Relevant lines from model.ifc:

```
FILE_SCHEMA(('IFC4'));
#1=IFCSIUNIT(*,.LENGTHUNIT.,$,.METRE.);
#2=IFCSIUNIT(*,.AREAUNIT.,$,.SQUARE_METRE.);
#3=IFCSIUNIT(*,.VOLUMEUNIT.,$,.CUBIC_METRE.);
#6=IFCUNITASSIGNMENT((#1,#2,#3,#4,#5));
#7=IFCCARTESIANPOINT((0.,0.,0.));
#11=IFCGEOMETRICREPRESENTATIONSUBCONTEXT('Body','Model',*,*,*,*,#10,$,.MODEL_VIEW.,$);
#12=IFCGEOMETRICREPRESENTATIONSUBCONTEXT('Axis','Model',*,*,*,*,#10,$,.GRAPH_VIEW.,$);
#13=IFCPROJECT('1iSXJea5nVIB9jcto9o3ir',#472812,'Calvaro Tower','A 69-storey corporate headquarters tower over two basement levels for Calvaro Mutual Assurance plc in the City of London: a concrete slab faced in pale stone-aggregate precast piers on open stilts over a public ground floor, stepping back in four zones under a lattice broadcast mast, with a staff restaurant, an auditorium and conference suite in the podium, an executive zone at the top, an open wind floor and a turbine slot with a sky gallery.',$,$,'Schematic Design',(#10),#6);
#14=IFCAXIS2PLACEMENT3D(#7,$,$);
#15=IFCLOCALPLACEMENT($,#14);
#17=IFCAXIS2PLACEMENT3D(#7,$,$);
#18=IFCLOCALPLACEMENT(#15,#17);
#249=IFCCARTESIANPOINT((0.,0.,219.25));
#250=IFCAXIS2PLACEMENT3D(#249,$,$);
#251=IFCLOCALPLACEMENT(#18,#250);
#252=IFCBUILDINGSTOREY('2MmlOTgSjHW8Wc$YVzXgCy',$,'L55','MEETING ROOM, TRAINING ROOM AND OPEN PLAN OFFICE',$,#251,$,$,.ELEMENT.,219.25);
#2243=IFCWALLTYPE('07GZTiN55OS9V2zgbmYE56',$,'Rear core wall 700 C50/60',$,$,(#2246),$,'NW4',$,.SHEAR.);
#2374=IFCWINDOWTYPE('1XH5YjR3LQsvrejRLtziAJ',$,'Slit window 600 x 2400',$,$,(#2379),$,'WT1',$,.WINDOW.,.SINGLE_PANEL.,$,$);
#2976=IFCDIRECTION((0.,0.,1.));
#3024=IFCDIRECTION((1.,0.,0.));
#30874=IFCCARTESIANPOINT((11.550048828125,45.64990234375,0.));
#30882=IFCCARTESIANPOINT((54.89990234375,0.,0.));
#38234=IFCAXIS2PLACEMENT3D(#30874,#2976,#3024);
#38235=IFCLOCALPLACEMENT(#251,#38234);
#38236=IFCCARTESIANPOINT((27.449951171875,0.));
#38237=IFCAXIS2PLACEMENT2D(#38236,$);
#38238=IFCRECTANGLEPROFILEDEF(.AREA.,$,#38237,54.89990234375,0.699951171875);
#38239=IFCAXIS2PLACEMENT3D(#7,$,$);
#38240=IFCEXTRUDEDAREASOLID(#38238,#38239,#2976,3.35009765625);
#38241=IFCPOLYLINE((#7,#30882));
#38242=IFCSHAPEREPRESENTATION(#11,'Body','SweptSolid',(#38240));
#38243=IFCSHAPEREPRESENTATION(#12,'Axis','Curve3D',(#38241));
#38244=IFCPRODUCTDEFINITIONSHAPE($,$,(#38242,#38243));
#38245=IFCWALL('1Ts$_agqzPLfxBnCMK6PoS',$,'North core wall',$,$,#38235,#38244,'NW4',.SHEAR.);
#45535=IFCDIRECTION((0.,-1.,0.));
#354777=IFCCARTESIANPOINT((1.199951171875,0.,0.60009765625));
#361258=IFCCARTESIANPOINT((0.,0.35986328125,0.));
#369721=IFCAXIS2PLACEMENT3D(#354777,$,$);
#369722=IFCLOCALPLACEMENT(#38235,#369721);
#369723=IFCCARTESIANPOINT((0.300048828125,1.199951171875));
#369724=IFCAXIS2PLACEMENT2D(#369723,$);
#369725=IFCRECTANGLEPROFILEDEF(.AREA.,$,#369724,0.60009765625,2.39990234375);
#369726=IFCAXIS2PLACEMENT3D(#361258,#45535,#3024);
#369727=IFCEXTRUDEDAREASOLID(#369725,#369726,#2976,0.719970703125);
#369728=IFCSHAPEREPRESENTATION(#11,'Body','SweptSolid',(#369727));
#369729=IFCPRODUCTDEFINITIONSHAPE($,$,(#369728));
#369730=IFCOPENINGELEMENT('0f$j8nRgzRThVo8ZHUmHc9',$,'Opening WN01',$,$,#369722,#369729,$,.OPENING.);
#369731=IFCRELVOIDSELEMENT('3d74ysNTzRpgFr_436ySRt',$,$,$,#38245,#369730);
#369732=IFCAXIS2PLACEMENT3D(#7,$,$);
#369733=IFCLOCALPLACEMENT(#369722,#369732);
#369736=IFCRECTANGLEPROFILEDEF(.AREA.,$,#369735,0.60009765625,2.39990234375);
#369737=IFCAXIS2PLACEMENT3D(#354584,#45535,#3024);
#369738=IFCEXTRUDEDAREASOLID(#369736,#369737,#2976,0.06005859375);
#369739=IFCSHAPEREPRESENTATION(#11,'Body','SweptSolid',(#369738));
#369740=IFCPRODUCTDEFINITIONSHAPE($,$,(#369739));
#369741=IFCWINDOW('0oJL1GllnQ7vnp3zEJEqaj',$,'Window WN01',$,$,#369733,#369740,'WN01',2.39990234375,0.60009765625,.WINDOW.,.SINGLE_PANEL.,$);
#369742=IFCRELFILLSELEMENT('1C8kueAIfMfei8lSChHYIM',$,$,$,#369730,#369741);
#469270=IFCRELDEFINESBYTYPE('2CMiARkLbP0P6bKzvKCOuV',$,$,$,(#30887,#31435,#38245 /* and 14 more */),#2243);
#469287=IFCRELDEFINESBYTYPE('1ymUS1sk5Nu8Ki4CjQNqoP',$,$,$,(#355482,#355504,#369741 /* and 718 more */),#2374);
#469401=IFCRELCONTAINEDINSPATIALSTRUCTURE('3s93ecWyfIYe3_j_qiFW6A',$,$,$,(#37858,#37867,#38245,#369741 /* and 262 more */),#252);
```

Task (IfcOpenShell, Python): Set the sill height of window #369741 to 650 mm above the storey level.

```python
import numpy as np
import ifcopenshell
import ifcopenshell.api.geometry
import ifcopenshell.geom
import ifcopenshell.util.element
import ifcopenshell.util.placement
import ifcopenshell.util.shape
import ifcopenshell.util.unit

model = ifcopenshell.open("model.ifc")
unit_scale = ifcopenshell.util.unit.calculate_unit_scale(model)

window = model.by_guid("0oJL1GllnQ7vnp3zEJEqaj")
opening = window.FillsVoids[0].RelatingOpeningElement
storey = ifcopenshell.util.element.get_container(window, ifc_class="IfcBuildingStorey")
level = ifcopenshell.util.placement.get_local_placement(storey.ObjectPlacement)[2, 3]

# The opening's origin need not be at the sill, so measure its lowest point.
shape = ifcopenshell.geom.create_shape(ifcopenshell.geom.settings(), opening)
bottom = ifcopenshell.util.shape.get_shape_bottom_elevation(shape, shape.geometry) / unit_scale
dz = level + 0.65 - bottom

shift = np.array([0.0, 0.0, dz])
# The window is placed relative to its opening, so it follows when the opening moves.
matrix = ifcopenshell.util.placement.get_local_placement(opening.ObjectPlacement)
matrix[:3, 3] += shift
ifcopenshell.api.geometry.edit_object_placement(
    model, product=opening, matrix=matrix, is_si=False, should_transform_children=True
)

print(f"moved by {dz * unit_scale:+.3f} m")

model.write("model_rev.ifc")
```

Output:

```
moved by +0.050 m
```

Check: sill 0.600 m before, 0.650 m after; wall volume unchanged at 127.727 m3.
